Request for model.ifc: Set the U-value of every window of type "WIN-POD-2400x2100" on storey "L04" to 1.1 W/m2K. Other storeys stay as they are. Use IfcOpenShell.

First a look at what the model holds.

```python
import ifcopenshell
import ifcopenshell.util.element

model = ifcopenshell.open("model.ifc")
print(model.schema)
storey = next(s for s in model.by_type("IfcBuildingStorey") if s.Name == "L04")
windows = [e for e in ifcopenshell.util.element.get_decomposition(storey) if e.is_a("IfcWindow")]
seen = {}
for e in windows:
    element_type = ifcopenshell.util.element.get_type(e)
    key = (element_type.Name if element_type != e and element_type else None, ifcopenshell.util.element.get_pset(e, "Pset_WindowCommon", "ThermalTransmittance"))
    seen[key] = seen.get(key, 0) + 1
for (name, value), count in sorted(seen.items(), key=str):
    print(count, "x", name, "|", value)
```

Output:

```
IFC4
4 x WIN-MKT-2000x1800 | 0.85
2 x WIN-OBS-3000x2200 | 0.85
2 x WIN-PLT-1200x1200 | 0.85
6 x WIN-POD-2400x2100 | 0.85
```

```python
import ifcopenshell
import ifcopenshell.api.pset
import ifcopenshell.util.element

model = ifcopenshell.open("model.ifc")

storey = next(s for s in model.by_type("IfcBuildingStorey") if s.Name == "L04")
windows = [e for e in ifcopenshell.util.element.get_decomposition(storey) if e.is_a("IfcWindow")]

count = 0
for e in windows:
    element_type = ifcopenshell.util.element.get_type(e)
    if element_type in (None, e) or element_type.Name != "WIN-POD-2400x2100":
        continue
    # add_pset returns the element's existing set when there is one.
    pset = ifcopenshell.api.pset.add_pset(model, product=e, name="Pset_WindowCommon")
    ifcopenshell.api.pset.edit_pset(model, pset=pset, properties={"ThermalTransmittance": 1.1})
    count += 1

print(count, "windows updated")

model.write("model_v2.ifc")
```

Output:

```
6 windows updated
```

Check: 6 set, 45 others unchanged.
